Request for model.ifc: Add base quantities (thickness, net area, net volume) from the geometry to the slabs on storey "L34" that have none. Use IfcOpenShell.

First a look at what the model holds.

```python
import ifcopenshell
import ifcopenshell.util.element
import ifcopenshell.util.unit

model = ifcopenshell.open("model.ifc")
print(model.schema)
for unit_type in ("LENGTHUNIT", "AREAUNIT", "VOLUMEUNIT"):
    print(unit_type, ifcopenshell.util.unit.calculate_unit_scale(model, unit_type))
storey = next(s for s in model.by_type("IfcBuildingStorey") if s.Name == "L34")
slabs = [e for e in ifcopenshell.util.element.get_decomposition(storey) if e.is_a("IfcSlab")]
for e in sorted(slabs, key=lambda e: e.id()):
    print(e.id(), e.is_a(), e.Name, list(ifcopenshell.util.element.get_psets(e, qtos_only=True)), sep=" | ")
```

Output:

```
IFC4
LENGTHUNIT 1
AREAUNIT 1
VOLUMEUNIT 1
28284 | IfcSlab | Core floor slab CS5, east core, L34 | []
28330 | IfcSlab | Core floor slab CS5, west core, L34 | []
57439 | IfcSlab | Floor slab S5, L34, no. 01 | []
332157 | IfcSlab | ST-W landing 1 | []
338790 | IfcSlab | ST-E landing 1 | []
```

```python
import ifcopenshell
import ifcopenshell.api.pset
import ifcopenshell.geom
import ifcopenshell.util.element
import ifcopenshell.util.shape
import ifcopenshell.util.unit

model = ifcopenshell.open("model.ifc")
unit_scale = ifcopenshell.util.unit.calculate_unit_scale(model)
area_scale = ifcopenshell.util.unit.calculate_unit_scale(model, "AREAUNIT")
volume_scale = ifcopenshell.util.unit.calculate_unit_scale(model, "VOLUMEUNIT")
settings = ifcopenshell.geom.settings()

storey = next(s for s in model.by_type("IfcBuildingStorey") if s.Name == "L34")
slabs = [e for e in ifcopenshell.util.element.get_decomposition(storey) if e.is_a("IfcSlab")]

for e in sorted(slabs, key=lambda e: e.id()):
    if ifcopenshell.util.element.get_psets(e, qtos_only=True, should_inherit=False):
        continue
    # Geometry comes back in metres, in the element's own axes.
    shape = ifcopenshell.geom.create_shape(settings, e)
    values = {
        "Width": ifcopenshell.util.shape.get_z(shape.geometry) / unit_scale,
        "NetArea": ifcopenshell.util.shape.get_footprint_area(shape.geometry) / area_scale,
        "NetVolume": ifcopenshell.util.shape.get_volume(shape.geometry) / volume_scale,
    }
    qto = ifcopenshell.api.pset.add_qto(model, product=e, name="Qto_SlabBaseQuantities")
    ifcopenshell.api.pset.edit_qto(model, qto=qto, properties=values)
    print(e.id(), {k: round(v, 3) for k, v in values.items()})

model.write("model-out.ifc")
```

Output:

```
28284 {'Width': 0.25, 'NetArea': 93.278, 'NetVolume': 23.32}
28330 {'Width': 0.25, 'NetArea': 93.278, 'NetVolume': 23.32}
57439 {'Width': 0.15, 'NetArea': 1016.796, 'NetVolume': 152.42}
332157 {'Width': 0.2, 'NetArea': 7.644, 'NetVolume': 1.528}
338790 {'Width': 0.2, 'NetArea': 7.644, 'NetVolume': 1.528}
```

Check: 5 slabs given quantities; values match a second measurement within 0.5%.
